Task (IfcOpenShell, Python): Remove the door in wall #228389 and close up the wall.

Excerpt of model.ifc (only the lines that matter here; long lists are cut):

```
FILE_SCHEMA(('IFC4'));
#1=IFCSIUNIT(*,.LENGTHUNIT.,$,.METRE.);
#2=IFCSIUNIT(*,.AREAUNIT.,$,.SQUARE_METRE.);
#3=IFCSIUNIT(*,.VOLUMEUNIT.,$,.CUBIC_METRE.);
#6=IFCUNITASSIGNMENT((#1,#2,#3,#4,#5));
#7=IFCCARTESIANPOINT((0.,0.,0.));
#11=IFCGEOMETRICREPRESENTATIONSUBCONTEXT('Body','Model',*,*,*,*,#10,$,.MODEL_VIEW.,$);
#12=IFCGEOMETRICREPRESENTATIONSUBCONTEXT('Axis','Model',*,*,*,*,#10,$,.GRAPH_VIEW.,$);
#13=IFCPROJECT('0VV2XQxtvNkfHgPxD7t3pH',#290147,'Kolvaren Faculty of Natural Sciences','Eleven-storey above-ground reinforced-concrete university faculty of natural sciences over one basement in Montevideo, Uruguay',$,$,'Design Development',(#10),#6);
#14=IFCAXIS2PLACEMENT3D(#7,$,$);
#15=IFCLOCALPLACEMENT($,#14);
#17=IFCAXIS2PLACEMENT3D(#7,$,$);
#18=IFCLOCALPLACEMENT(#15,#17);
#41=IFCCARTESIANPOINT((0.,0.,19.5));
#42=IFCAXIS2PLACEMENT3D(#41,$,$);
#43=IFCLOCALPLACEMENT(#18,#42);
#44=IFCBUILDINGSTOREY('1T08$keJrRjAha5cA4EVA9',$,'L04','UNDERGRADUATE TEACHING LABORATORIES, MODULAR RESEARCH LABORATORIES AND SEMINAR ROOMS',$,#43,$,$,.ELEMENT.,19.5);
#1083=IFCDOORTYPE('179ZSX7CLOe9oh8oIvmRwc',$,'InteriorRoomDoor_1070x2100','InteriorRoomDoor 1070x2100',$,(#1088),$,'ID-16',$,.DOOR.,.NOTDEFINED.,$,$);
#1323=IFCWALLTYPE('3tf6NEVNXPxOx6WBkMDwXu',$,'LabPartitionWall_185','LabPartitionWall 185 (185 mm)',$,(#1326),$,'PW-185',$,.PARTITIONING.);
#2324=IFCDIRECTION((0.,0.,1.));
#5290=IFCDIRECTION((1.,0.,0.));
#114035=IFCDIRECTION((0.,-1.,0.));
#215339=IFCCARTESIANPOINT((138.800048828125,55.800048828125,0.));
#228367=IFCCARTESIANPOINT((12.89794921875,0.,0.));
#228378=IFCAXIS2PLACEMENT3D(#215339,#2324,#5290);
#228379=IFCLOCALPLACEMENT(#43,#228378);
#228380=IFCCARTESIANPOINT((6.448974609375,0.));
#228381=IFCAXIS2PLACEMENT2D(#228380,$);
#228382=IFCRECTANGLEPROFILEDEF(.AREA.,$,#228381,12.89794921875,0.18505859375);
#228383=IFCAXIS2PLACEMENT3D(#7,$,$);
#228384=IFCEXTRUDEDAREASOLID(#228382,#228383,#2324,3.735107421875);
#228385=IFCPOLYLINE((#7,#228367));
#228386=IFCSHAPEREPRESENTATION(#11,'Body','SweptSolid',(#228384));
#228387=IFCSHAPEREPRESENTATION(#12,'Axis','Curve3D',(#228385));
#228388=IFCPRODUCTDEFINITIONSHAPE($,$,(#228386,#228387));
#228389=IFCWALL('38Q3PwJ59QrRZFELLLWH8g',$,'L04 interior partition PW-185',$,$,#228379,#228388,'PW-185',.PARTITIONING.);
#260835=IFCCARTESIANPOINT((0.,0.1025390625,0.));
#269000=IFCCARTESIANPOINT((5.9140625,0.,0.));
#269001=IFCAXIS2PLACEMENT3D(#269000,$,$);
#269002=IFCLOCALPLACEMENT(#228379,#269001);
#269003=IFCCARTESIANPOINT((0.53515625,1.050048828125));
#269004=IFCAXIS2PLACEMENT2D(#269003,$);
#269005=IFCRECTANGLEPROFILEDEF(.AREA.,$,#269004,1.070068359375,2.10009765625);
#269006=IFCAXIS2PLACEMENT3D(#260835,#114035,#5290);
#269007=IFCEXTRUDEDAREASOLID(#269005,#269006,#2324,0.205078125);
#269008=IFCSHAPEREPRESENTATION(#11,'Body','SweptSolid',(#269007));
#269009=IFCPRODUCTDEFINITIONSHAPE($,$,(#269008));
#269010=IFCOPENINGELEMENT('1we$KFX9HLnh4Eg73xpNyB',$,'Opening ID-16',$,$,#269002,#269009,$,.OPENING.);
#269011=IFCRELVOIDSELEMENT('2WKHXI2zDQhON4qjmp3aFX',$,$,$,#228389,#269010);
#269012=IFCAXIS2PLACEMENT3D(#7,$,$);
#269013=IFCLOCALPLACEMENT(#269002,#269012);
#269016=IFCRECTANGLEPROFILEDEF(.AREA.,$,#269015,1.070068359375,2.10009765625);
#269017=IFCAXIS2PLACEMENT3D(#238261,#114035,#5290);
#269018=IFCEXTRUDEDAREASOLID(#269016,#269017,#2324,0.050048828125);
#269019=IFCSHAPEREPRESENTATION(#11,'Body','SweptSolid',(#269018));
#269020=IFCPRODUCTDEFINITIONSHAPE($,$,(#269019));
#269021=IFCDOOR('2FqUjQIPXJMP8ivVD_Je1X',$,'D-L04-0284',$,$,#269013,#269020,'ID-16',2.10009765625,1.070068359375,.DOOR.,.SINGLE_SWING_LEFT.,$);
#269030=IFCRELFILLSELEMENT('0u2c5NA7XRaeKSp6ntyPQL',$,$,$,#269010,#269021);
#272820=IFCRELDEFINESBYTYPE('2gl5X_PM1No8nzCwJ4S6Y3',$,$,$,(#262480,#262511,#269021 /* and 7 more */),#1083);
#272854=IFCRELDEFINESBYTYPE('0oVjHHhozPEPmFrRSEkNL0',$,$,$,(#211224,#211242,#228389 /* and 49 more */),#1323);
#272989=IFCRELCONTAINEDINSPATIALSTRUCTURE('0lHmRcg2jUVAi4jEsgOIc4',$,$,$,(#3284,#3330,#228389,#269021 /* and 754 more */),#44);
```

```python
import ifcopenshell
import ifcopenshell.api.feature
import ifcopenshell.api.root
import ifcopenshell.geom
import ifcopenshell.util.shape

model = ifcopenshell.open("model.ifc")
settings = ifcopenshell.geom.settings()


def volume(element):
    """Net volume in cubic metres, openings subtracted."""
    shape = ifcopenshell.geom.create_shape(settings, element)
    return ifcopenshell.util.shape.get_volume(shape.geometry)


door = model.by_guid("2FqUjQIPXJMP8ivVD_Je1X")
opening = door.FillsVoids[0].RelatingOpeningElement
wall = opening.VoidsElements[0].RelatingBuildingElement
before = volume(wall)

ifcopenshell.api.root.remove_product(model, product=door)
ifcopenshell.api.feature.remove_feature(model, feature=opening)

after = volume(wall)

print(f"wall volume {before:.3f} -> {after:.3f} m3")

model.write("model-out.ifc")
```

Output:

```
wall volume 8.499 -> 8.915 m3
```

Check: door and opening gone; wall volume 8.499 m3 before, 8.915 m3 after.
